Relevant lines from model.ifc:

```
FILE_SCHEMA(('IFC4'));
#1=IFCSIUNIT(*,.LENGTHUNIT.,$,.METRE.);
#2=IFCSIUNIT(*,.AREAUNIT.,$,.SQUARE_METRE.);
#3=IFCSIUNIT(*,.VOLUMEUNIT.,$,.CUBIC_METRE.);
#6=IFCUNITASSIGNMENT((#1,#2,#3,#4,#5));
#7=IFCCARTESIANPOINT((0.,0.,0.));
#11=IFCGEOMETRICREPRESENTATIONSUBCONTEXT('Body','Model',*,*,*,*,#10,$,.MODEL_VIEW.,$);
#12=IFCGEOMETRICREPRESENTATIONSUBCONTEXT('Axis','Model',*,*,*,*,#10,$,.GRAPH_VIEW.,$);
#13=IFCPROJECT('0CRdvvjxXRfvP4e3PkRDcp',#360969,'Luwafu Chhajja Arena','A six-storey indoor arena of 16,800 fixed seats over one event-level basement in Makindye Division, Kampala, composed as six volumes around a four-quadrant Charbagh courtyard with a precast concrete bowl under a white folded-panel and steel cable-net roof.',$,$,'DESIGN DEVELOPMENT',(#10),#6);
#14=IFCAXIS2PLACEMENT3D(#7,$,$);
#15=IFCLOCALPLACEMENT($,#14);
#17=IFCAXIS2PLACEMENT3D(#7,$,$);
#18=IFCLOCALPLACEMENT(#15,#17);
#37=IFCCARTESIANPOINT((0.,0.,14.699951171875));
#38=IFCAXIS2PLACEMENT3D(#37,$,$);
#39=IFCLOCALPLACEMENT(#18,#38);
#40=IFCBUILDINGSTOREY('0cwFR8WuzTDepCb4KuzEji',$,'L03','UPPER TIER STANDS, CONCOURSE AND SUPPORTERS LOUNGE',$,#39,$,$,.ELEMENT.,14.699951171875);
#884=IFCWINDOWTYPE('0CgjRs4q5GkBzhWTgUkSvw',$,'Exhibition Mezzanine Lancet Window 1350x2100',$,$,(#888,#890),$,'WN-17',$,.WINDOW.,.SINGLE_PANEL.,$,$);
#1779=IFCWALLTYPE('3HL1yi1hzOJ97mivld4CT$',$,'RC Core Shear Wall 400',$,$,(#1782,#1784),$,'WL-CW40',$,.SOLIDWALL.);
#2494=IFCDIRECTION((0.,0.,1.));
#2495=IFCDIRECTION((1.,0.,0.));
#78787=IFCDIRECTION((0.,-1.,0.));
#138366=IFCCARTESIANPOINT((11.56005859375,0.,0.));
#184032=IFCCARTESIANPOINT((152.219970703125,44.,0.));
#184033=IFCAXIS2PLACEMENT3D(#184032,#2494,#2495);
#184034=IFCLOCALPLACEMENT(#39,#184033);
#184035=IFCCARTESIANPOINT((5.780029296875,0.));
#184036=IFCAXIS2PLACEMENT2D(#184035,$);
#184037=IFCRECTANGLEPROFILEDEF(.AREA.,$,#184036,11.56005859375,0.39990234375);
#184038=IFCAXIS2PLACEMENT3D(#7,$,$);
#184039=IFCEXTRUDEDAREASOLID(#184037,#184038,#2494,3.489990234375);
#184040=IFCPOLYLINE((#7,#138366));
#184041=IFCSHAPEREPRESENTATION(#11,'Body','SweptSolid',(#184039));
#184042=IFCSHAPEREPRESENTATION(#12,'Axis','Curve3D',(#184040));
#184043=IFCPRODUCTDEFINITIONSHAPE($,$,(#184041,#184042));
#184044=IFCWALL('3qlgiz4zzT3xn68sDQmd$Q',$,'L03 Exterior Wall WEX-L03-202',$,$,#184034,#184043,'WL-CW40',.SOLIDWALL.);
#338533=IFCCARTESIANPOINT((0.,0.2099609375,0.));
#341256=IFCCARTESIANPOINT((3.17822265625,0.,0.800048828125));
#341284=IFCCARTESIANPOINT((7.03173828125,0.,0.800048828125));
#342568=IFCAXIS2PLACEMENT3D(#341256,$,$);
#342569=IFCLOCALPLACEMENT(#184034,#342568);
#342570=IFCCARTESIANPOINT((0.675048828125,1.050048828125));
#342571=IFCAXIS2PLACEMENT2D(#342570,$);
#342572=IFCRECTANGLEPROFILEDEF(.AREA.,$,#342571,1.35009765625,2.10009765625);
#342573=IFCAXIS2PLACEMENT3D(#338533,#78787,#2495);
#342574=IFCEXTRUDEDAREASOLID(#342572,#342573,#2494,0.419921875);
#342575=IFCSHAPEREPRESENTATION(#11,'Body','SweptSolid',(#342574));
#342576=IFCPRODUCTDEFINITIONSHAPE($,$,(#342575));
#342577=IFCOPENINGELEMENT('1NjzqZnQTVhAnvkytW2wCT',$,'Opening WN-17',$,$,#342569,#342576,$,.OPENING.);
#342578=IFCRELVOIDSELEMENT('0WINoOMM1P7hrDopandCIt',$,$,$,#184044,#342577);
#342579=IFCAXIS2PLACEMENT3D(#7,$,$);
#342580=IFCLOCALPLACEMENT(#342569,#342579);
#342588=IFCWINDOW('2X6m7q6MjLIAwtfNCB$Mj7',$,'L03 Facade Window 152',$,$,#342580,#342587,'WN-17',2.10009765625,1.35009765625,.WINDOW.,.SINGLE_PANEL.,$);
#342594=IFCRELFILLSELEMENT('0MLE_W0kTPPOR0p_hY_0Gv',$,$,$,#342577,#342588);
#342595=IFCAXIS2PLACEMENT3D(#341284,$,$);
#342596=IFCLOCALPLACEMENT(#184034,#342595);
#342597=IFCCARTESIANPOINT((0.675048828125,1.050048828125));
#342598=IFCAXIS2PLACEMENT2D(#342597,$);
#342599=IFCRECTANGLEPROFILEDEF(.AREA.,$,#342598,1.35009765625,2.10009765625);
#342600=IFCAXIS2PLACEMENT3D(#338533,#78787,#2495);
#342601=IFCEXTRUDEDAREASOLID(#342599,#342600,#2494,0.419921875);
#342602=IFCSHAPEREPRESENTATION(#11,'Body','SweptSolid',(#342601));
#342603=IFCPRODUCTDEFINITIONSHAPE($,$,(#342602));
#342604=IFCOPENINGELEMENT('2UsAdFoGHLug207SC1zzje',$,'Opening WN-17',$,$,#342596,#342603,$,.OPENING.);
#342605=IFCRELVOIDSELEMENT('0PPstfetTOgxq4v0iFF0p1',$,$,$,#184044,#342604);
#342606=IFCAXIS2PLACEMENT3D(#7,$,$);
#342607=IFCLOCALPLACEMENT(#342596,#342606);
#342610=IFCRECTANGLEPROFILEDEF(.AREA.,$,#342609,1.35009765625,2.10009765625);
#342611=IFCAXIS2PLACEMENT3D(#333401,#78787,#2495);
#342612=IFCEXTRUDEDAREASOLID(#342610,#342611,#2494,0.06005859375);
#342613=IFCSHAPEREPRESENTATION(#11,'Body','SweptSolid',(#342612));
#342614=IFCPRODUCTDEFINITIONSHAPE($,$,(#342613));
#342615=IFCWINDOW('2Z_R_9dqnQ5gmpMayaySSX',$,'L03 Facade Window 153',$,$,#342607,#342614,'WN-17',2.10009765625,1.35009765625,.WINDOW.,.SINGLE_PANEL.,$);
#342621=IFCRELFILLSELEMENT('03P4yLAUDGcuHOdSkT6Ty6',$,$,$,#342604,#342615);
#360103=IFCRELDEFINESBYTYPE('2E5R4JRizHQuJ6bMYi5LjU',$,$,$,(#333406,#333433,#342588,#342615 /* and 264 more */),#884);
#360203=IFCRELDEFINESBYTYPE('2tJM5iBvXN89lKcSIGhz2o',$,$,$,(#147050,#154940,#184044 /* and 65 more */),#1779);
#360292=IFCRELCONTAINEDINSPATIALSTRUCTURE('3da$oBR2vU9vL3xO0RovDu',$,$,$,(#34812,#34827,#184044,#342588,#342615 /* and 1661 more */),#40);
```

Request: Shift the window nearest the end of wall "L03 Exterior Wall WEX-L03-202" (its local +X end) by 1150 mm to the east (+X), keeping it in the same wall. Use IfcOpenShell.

```python
import ifcopenshell
import ifcopenshell.api.geometry
import ifcopenshell.util.placement
import ifcopenshell.util.unit

model = ifcopenshell.open("model.ifc")
unit_scale = ifcopenshell.util.unit.calculate_unit_scale(model)

window = model.by_guid("2Z_R_9dqnQ5gmpMayaySSX")
opening = window.FillsVoids[0].RelatingOpeningElement
wall = opening.VoidsElements[0].RelatingBuildingElement

wall_matrix = ifcopenshell.util.placement.get_local_placement(wall.ObjectPlacement)
shift = wall_matrix[:3, 0] * 1.15 / unit_scale
before = ifcopenshell.util.placement.get_local_placement(window.ObjectPlacement)[:3, 3].copy()

# The window is placed relative to its opening, so it follows when the opening moves.
matrix = ifcopenshell.util.placement.get_local_placement(opening.ObjectPlacement)
matrix[:3, 3] += shift
ifcopenshell.api.geometry.edit_object_placement(
    model, product=opening, matrix=matrix, is_si=False, should_transform_children=True
)

after = ifcopenshell.util.placement.get_local_placement(window.ObjectPlacement)[:3, 3]
print("window moved by", (after - before).round(3) + 0.0)

model.write("model-out.ifc")
```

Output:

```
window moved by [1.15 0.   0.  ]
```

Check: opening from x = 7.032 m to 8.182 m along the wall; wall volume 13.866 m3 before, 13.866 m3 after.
